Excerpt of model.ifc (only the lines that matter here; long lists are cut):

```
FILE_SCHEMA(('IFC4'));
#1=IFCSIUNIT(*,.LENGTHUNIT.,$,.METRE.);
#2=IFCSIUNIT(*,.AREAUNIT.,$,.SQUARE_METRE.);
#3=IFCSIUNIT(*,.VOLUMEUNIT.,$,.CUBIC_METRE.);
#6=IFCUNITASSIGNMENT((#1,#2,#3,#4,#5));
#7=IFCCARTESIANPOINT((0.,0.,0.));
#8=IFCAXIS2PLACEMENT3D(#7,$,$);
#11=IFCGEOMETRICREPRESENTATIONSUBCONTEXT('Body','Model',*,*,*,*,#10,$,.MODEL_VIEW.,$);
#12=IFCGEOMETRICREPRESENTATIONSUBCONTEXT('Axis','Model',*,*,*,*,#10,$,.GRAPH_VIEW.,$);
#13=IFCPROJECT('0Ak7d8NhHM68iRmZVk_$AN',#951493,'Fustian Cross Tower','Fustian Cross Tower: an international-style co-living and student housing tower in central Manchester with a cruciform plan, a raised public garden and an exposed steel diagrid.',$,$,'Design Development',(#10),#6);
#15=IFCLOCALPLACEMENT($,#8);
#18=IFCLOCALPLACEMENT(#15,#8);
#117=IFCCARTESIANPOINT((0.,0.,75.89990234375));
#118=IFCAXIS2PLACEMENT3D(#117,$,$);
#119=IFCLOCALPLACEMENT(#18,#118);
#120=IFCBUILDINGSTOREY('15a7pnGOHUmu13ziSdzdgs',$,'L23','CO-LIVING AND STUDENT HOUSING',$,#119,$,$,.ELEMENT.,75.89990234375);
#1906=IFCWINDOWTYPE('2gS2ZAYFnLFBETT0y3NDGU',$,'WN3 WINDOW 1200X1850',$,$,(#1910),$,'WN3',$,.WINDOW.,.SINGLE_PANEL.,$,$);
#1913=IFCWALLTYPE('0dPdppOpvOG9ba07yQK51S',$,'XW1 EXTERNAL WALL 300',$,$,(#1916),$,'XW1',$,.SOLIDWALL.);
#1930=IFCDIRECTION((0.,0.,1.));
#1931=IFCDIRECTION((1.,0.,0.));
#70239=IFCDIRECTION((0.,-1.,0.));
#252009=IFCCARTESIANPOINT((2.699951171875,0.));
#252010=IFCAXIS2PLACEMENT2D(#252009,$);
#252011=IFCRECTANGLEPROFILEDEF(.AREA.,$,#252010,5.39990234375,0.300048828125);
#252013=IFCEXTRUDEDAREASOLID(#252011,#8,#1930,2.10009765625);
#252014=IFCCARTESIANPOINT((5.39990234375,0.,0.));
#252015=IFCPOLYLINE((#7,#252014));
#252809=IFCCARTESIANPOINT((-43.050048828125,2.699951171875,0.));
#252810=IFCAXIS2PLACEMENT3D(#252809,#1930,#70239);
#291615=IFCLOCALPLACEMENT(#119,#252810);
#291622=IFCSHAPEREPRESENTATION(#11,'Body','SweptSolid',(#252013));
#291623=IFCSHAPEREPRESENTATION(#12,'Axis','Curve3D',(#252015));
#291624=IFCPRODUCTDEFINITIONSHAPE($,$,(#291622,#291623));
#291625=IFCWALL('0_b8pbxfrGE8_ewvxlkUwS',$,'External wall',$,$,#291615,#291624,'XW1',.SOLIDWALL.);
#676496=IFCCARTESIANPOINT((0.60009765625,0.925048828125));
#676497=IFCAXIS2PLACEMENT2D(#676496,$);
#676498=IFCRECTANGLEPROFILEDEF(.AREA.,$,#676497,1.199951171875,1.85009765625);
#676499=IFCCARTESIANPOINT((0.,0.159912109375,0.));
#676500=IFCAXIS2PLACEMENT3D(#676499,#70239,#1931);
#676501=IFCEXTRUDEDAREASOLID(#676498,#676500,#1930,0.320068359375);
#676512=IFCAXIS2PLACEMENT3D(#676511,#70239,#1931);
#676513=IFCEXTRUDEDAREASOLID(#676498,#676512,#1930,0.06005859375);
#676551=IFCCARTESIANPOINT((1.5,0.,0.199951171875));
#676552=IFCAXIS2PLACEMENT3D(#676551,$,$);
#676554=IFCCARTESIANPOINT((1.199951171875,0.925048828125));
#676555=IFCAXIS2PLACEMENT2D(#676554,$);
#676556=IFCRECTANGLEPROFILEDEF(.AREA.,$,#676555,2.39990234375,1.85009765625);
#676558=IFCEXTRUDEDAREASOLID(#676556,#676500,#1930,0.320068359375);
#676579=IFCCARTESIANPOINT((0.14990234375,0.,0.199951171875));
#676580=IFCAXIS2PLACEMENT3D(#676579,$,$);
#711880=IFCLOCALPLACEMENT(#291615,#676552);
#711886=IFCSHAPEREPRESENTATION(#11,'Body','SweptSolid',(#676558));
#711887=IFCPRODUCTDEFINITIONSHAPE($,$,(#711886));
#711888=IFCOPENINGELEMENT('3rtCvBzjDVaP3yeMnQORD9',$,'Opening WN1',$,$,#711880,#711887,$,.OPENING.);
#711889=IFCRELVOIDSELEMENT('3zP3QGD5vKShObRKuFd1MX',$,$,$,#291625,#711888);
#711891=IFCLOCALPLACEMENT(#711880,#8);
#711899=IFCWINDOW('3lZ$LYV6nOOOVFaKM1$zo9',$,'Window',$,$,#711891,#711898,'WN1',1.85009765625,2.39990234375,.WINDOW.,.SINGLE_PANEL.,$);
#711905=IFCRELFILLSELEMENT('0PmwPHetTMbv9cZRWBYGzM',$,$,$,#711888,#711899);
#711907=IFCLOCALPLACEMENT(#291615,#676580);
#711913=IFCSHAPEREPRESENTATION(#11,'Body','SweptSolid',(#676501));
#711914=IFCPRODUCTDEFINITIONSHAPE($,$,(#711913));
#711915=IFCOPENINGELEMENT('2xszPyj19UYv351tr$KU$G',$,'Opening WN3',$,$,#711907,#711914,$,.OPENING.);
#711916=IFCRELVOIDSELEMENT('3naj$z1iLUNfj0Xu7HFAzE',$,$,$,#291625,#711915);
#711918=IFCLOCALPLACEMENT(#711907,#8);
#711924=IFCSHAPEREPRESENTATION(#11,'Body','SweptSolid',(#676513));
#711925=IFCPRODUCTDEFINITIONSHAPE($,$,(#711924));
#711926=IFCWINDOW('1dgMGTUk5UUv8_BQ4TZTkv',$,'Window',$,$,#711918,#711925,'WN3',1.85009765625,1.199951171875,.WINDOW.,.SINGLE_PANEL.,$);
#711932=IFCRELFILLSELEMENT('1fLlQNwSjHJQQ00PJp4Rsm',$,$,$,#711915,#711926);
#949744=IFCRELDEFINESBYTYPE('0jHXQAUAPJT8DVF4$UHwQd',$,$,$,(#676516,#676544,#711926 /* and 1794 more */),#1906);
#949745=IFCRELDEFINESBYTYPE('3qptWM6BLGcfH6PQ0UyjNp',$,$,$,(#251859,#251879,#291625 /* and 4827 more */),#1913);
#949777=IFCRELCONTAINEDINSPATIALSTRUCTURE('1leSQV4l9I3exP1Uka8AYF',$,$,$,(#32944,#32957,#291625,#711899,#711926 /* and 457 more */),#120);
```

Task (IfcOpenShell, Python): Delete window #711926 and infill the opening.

```python
import ifcopenshell
import ifcopenshell.api.feature
import ifcopenshell.api.root
import ifcopenshell.geom
import ifcopenshell.util.shape

model = ifcopenshell.open("model.ifc")
settings = ifcopenshell.geom.settings()


def volume(element):
    """Net volume in cubic metres, openings subtracted."""
    shape = ifcopenshell.geom.create_shape(settings, element)
    return ifcopenshell.util.shape.get_volume(shape.geometry)


window = model.by_guid("1dgMGTUk5UUv8_BQ4TZTkv")
opening = window.FillsVoids[0].RelatingOpeningElement
wall = opening.VoidsElements[0].RelatingBuildingElement
before = volume(wall)

ifcopenshell.api.root.remove_product(model, product=window)
ifcopenshell.api.feature.remove_feature(model, feature=opening)

after = volume(wall)

print(f"wall volume {before:.3f} -> {after:.3f} m3")

model.write("model_v2.ifc")
```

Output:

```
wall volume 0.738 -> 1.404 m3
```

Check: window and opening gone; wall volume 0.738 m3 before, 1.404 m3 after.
